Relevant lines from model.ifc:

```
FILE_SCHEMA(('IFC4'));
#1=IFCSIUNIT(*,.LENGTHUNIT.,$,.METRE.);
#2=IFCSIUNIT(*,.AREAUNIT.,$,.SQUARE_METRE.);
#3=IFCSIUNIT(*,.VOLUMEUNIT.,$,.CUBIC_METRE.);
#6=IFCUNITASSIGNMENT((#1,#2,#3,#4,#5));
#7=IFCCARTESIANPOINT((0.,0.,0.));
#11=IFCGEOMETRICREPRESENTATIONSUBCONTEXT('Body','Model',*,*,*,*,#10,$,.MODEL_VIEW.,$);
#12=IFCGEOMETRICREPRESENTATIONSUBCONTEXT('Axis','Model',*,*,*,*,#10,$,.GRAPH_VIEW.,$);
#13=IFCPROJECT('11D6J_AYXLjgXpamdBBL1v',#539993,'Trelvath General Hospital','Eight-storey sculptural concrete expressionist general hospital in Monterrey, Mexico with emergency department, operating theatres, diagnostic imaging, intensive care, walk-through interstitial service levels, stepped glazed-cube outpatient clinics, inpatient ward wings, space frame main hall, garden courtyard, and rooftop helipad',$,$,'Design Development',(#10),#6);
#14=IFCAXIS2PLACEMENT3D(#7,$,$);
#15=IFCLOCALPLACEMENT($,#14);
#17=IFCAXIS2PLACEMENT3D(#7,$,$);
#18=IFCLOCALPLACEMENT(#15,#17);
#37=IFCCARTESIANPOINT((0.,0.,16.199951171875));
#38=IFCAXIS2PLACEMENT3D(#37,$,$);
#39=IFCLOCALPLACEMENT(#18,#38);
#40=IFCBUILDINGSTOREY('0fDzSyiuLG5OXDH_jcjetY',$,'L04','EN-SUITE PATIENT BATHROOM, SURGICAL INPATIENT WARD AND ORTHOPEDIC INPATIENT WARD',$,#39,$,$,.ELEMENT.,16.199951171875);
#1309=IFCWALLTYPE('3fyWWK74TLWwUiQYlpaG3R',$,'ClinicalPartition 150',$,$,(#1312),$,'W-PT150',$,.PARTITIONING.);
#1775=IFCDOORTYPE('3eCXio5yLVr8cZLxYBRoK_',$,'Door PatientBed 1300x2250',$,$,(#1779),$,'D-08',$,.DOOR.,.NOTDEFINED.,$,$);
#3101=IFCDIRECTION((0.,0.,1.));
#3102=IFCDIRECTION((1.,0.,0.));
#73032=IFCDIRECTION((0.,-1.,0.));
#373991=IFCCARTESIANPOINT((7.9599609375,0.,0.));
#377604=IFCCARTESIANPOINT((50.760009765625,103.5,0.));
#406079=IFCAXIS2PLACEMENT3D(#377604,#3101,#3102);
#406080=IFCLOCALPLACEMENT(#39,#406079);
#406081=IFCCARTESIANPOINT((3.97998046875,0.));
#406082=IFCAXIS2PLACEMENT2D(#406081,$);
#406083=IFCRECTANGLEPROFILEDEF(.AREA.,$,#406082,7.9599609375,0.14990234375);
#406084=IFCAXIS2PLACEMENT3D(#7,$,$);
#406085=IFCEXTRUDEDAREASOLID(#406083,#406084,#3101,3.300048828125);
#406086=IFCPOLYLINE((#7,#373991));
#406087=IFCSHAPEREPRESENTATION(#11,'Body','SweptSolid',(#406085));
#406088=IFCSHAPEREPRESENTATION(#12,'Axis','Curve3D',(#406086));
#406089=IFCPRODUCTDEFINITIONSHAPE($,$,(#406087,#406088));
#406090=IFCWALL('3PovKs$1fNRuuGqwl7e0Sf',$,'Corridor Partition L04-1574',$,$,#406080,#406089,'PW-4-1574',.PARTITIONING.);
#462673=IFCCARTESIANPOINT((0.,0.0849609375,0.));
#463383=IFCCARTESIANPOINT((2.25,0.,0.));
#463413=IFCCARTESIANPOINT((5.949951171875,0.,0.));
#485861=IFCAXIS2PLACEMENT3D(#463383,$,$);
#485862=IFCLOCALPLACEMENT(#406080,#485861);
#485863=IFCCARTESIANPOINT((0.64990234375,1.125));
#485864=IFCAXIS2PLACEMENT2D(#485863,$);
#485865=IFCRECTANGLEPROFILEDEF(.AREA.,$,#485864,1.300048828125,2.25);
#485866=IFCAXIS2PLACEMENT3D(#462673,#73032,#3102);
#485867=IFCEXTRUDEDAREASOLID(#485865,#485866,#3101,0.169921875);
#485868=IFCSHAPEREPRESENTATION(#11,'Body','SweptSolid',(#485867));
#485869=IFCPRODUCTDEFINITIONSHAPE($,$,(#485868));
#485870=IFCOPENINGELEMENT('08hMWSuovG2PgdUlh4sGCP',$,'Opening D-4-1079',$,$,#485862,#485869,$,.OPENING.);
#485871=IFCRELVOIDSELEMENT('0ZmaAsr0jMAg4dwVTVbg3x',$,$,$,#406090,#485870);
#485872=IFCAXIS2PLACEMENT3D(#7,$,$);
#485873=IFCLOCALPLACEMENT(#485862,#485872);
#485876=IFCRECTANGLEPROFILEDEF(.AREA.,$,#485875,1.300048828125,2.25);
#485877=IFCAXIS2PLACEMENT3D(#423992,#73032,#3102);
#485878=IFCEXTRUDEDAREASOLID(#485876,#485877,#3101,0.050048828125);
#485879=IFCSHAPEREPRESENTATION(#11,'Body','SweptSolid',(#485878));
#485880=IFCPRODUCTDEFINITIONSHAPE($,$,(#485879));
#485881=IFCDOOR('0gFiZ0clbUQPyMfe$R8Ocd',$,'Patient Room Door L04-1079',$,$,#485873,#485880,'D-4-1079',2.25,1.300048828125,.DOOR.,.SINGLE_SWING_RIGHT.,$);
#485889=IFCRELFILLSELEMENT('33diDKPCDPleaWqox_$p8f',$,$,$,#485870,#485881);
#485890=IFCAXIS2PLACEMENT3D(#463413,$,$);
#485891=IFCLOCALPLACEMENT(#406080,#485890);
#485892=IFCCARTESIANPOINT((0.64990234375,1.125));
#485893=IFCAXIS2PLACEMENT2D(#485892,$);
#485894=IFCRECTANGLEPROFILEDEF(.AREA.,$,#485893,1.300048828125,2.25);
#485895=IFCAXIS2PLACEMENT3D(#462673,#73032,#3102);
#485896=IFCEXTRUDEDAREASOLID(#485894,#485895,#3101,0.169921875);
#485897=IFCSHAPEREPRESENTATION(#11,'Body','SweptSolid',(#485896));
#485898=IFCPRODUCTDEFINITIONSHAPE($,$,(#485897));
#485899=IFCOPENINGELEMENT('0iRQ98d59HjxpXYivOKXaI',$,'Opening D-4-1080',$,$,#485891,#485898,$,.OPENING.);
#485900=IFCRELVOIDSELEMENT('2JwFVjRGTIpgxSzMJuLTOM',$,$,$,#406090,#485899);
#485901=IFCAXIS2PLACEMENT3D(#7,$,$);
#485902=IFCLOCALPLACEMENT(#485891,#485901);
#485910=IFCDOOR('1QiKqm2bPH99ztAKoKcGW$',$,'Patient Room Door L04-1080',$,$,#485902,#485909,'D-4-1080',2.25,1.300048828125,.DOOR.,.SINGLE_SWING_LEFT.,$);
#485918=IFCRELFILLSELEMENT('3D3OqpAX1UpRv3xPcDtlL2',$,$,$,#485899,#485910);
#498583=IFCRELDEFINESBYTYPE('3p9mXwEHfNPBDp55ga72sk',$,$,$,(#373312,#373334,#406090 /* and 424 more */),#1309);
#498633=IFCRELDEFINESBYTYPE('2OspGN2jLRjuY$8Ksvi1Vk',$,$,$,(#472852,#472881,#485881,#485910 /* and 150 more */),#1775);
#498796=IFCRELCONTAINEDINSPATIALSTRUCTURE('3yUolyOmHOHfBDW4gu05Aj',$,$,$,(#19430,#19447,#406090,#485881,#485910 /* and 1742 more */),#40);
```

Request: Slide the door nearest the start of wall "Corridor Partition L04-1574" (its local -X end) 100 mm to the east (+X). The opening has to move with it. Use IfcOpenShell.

```python
import ifcopenshell
import ifcopenshell.api.geometry
import ifcopenshell.util.placement

model = ifcopenshell.open("model.ifc")

door = model.by_guid("0gFiZ0clbUQPyMfe$R8Ocd")
opening = door.FillsVoids[0].RelatingOpeningElement
wall = opening.VoidsElements[0].RelatingBuildingElement

wall_matrix = ifcopenshell.util.placement.get_local_placement(wall.ObjectPlacement)
shift = wall_matrix[:3, 0] * 0.1
before = ifcopenshell.util.placement.get_local_placement(door.ObjectPlacement)[:3, 3].copy()

# The door is placed relative to its opening, so it follows when the opening moves.
matrix = ifcopenshell.util.placement.get_local_placement(opening.ObjectPlacement)
matrix[:3, 3] += shift
ifcopenshell.api.geometry.edit_object_placement(
    model, product=opening, matrix=matrix, is_si=False, should_transform_children=True
)

after = ifcopenshell.util.placement.get_local_placement(door.ObjectPlacement)[:3, 3]
print("door moved by", (after - before).round(3) + 0.0)

model.write("model_edited.ifc")
```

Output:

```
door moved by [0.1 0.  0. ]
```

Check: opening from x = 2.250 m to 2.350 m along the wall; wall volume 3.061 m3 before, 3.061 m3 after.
